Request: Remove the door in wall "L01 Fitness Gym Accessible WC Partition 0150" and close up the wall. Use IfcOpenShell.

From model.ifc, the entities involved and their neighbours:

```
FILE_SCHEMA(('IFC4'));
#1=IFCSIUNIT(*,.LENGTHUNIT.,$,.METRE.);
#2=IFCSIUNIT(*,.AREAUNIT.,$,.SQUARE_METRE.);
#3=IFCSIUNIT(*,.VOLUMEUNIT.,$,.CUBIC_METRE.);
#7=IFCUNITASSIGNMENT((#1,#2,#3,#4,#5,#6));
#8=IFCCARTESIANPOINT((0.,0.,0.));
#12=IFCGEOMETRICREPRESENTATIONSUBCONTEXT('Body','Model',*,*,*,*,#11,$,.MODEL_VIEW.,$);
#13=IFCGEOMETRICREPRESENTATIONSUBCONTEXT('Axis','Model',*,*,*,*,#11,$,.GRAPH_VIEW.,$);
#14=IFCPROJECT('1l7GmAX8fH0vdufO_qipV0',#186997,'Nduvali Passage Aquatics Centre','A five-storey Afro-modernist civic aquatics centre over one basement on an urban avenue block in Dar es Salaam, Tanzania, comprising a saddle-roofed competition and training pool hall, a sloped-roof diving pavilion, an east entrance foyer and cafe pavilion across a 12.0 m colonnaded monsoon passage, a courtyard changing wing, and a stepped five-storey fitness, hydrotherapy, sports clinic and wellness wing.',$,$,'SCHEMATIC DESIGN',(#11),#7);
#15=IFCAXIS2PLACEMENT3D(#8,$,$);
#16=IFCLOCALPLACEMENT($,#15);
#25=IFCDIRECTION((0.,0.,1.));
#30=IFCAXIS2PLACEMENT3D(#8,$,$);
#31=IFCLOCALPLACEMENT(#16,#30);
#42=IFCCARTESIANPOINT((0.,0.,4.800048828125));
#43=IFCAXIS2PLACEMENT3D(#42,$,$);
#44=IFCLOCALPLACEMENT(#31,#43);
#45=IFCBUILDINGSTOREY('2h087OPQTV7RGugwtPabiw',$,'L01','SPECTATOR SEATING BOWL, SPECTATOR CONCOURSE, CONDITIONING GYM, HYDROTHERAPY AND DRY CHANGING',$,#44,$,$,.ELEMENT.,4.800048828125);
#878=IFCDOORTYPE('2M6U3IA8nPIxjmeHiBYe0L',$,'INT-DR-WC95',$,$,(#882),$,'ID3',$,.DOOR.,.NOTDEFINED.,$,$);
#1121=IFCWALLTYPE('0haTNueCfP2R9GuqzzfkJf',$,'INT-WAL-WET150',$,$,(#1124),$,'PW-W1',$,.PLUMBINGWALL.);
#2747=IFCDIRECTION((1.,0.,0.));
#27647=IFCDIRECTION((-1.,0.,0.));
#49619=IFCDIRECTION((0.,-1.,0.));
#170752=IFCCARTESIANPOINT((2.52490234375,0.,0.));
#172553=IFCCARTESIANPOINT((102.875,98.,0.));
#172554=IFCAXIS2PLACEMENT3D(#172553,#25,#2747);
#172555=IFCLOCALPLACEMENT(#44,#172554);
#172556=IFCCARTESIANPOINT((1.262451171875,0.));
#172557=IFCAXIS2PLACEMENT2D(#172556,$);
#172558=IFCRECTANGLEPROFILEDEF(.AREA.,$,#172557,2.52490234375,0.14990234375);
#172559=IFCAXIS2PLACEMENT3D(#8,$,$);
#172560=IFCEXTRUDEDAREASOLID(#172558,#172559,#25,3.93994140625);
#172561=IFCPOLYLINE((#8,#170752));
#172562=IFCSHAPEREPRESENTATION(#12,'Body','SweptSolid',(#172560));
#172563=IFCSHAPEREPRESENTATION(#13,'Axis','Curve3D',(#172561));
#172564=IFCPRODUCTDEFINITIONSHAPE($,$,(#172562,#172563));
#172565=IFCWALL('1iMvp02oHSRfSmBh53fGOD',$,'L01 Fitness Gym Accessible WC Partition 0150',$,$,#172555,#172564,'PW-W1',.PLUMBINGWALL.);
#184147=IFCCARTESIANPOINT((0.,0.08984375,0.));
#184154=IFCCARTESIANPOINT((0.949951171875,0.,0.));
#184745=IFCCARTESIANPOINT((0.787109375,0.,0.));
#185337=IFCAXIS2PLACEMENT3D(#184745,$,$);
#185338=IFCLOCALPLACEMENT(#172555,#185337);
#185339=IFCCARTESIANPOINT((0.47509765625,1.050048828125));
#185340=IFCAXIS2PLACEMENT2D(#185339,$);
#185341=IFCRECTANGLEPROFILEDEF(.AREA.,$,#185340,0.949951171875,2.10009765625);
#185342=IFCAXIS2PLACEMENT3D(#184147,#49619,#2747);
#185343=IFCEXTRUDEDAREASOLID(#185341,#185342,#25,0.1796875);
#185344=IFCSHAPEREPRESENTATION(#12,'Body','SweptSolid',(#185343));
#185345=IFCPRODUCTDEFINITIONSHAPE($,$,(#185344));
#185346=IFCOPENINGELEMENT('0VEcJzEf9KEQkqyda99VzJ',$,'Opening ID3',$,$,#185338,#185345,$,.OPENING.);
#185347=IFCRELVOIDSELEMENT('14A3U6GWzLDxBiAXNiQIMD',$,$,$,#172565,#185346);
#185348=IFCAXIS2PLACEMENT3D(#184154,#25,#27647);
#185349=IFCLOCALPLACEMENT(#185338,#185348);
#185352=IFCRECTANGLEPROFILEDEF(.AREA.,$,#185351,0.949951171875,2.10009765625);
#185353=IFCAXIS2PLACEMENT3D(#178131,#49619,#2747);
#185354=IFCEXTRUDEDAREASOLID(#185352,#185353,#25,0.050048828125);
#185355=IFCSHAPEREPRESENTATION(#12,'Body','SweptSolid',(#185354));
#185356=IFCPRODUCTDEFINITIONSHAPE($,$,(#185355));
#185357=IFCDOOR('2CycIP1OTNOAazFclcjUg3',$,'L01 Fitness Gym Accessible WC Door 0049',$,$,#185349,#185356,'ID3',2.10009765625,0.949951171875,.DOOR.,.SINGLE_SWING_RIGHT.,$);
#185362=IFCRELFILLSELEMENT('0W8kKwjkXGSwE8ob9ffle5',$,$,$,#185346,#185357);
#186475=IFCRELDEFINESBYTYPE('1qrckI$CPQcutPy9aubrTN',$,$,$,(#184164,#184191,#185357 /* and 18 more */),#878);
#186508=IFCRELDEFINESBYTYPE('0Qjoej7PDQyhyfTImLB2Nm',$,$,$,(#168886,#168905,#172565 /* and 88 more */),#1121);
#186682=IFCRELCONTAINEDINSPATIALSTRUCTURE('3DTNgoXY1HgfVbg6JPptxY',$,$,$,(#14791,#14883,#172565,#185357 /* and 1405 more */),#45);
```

```python
import ifcopenshell
import ifcopenshell.api.feature
import ifcopenshell.api.root
import ifcopenshell.geom
import ifcopenshell.util.shape

model = ifcopenshell.open("model.ifc")
settings = ifcopenshell.geom.settings()


def volume(element):
    """Net volume in cubic metres, openings subtracted."""
    shape = ifcopenshell.geom.create_shape(settings, element)
    return ifcopenshell.util.shape.get_volume(shape.geometry)


door = model.by_guid("2CycIP1OTNOAazFclcjUg3")
opening = door.FillsVoids[0].RelatingOpeningElement
wall = opening.VoidsElements[0].RelatingBuildingElement
before = volume(wall)

ifcopenshell.api.root.remove_product(model, product=door)
ifcopenshell.api.feature.remove_feature(model, feature=opening)

after = volume(wall)

print(f"wall volume {before:.3f} -> {after:.3f} m3")

model.write("model_updated.ifc")
```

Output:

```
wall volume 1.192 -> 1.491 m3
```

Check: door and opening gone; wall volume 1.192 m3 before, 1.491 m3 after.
